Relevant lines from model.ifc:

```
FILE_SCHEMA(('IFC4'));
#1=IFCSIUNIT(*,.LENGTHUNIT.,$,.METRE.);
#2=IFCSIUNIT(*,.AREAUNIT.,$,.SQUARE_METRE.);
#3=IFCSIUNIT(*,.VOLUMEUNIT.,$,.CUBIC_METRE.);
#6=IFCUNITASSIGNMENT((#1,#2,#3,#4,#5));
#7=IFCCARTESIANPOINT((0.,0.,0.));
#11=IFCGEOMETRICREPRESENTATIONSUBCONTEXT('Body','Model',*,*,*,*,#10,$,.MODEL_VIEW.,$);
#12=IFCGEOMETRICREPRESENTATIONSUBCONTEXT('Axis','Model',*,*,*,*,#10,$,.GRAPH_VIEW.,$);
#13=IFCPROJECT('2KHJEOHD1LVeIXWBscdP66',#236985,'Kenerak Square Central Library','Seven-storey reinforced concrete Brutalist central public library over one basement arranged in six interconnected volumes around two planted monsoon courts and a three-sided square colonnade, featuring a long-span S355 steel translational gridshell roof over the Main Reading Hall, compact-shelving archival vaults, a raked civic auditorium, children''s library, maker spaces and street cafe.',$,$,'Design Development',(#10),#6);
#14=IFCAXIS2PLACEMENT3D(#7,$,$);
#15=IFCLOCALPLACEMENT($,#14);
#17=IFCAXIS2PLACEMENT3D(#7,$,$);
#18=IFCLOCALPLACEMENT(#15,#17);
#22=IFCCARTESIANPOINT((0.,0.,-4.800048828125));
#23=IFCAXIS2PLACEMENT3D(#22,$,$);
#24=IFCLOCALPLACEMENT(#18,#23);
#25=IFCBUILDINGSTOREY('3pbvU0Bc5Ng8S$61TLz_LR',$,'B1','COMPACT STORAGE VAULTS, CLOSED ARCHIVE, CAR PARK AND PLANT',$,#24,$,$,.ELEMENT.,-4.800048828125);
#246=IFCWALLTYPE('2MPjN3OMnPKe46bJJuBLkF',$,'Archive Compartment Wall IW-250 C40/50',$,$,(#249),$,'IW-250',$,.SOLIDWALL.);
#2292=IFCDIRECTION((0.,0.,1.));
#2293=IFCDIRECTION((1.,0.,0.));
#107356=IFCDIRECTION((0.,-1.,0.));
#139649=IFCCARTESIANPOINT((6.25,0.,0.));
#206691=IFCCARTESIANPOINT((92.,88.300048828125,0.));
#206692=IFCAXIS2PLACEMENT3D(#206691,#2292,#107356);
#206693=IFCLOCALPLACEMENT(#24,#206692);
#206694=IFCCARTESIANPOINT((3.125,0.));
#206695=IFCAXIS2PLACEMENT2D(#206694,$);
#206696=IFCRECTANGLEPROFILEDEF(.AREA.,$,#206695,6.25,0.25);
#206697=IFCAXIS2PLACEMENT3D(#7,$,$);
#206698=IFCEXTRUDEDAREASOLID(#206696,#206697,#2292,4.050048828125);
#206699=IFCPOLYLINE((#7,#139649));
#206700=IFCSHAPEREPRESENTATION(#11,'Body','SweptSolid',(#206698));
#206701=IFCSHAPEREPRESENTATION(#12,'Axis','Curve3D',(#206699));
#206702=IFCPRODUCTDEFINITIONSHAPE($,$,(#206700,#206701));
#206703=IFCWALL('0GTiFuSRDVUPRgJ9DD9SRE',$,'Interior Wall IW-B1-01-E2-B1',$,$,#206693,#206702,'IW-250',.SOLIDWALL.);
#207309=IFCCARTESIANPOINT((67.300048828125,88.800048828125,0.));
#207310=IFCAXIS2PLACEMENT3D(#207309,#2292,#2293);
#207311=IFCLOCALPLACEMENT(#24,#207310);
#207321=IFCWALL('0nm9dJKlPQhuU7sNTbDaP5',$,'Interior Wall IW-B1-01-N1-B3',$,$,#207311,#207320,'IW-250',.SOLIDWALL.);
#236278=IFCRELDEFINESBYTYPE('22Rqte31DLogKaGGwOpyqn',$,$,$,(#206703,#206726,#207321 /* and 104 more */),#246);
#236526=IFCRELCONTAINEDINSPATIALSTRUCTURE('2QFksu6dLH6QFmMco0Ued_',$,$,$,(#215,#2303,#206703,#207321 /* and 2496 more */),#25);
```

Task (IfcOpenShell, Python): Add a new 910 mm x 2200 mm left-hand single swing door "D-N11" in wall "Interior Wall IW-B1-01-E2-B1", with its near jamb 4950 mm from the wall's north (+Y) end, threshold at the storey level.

```python
import numpy as np
import ifcopenshell
import ifcopenshell.api.feature
import ifcopenshell.api.geometry
import ifcopenshell.api.root
import ifcopenshell.api.spatial
import ifcopenshell.geom
import ifcopenshell.util.element
import ifcopenshell.util.placement
import ifcopenshell.util.representation
import ifcopenshell.util.shape
import ifcopenshell.util.unit

model = ifcopenshell.open("model.ifc")
unit_scale = ifcopenshell.util.unit.calculate_unit_scale(model)
settings = ifcopenshell.geom.settings()


def volume(element):
    """Net volume in cubic metres, openings subtracted."""
    shape = ifcopenshell.geom.create_shape(settings, element)
    return ifcopenshell.util.shape.get_volume(shape.geometry)


wall = model.by_guid("0GTiFuSRDVUPRgJ9DD9SRE")
storey = ifcopenshell.util.element.get_container(wall, ifc_class="IfcBuildingStorey")
context = ifcopenshell.util.representation.get_context(model, "Model", "Body", "MODEL_VIEW")
before = volume(wall)

width, height, from_end, sill = 0.91, 2.2, 4.95, 0.0  # metres

# The wall runs along its own X axis, and the end named is its -X end.
wall_shape = ifcopenshell.geom.create_shape(settings, wall)
x, y, z = ifcopenshell.util.shape.get_vertices(wall_shape.geometry).T
start = x.min() + from_end
face, thickness = float(y.min()), float(y.max() - y.min())
wall_matrix = ifcopenshell.util.placement.get_local_placement(wall.ObjectPlacement)
level = ifcopenshell.util.placement.get_local_placement(storey.ObjectPlacement)[2, 3]


def in_wall(x, y):
    """Placement at x, y metres in the wall's axes, at sill height."""
    matrix = wall_matrix.copy()
    matrix[:, 3] = wall_matrix @ np.array([x / unit_scale, y / unit_scale, 0.0, 1.0])
    matrix[2, 3] = level + sill / unit_scale
    return matrix


# Opening: a box that overshoots both wall faces by 50 mm.
opening = ifcopenshell.api.root.create_entity(model, ifc_class="IfcOpeningElement", predefined_type="OPENING")
box = ifcopenshell.api.geometry.add_wall_representation(
    model, context=context, length=width, height=height, thickness=thickness + 0.1
)
ifcopenshell.api.geometry.assign_representation(model, product=opening, representation=box)
ifcopenshell.api.geometry.edit_object_placement(model, product=opening, matrix=in_wall(start, face - 0.05), is_si=False)
ifcopenshell.api.feature.add_feature(model, feature=opening, element=wall)

door = ifcopenshell.api.root.create_entity(model, ifc_class="IfcDoor", name="D-N11", predefined_type="DOOR")
door.OverallWidth, door.OverallHeight = width / unit_scale, height / unit_scale
door.OperationType = "SINGLE_SWING_LEFT"
body = ifcopenshell.api.geometry.add_door_representation(
    model,
    context=context,
    overall_width=door.OverallWidth,
    overall_height=door.OverallHeight,
    operation_type="SINGLE_SWING_LEFT",
    lining_properties={"LiningDepth": thickness / unit_scale, "ThresholdDepth": thickness / unit_scale},
)
ifcopenshell.api.geometry.assign_representation(model, product=door, representation=body)
ifcopenshell.api.spatial.assign_container(model, products=[door], relating_structure=storey)
ifcopenshell.api.feature.add_filling(model, opening=opening, element=door)

# The lining spans the wall, so the door starts at the wall face.
ifcopenshell.api.geometry.edit_object_placement(model, product=door, matrix=in_wall(start, face), is_si=False)

after = volume(wall)

print(f"wall volume {before:.3f} -> {after:.3f} m3")

model.write("model-out.ifc")
```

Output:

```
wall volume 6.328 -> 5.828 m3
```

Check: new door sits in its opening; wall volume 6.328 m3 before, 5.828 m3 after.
